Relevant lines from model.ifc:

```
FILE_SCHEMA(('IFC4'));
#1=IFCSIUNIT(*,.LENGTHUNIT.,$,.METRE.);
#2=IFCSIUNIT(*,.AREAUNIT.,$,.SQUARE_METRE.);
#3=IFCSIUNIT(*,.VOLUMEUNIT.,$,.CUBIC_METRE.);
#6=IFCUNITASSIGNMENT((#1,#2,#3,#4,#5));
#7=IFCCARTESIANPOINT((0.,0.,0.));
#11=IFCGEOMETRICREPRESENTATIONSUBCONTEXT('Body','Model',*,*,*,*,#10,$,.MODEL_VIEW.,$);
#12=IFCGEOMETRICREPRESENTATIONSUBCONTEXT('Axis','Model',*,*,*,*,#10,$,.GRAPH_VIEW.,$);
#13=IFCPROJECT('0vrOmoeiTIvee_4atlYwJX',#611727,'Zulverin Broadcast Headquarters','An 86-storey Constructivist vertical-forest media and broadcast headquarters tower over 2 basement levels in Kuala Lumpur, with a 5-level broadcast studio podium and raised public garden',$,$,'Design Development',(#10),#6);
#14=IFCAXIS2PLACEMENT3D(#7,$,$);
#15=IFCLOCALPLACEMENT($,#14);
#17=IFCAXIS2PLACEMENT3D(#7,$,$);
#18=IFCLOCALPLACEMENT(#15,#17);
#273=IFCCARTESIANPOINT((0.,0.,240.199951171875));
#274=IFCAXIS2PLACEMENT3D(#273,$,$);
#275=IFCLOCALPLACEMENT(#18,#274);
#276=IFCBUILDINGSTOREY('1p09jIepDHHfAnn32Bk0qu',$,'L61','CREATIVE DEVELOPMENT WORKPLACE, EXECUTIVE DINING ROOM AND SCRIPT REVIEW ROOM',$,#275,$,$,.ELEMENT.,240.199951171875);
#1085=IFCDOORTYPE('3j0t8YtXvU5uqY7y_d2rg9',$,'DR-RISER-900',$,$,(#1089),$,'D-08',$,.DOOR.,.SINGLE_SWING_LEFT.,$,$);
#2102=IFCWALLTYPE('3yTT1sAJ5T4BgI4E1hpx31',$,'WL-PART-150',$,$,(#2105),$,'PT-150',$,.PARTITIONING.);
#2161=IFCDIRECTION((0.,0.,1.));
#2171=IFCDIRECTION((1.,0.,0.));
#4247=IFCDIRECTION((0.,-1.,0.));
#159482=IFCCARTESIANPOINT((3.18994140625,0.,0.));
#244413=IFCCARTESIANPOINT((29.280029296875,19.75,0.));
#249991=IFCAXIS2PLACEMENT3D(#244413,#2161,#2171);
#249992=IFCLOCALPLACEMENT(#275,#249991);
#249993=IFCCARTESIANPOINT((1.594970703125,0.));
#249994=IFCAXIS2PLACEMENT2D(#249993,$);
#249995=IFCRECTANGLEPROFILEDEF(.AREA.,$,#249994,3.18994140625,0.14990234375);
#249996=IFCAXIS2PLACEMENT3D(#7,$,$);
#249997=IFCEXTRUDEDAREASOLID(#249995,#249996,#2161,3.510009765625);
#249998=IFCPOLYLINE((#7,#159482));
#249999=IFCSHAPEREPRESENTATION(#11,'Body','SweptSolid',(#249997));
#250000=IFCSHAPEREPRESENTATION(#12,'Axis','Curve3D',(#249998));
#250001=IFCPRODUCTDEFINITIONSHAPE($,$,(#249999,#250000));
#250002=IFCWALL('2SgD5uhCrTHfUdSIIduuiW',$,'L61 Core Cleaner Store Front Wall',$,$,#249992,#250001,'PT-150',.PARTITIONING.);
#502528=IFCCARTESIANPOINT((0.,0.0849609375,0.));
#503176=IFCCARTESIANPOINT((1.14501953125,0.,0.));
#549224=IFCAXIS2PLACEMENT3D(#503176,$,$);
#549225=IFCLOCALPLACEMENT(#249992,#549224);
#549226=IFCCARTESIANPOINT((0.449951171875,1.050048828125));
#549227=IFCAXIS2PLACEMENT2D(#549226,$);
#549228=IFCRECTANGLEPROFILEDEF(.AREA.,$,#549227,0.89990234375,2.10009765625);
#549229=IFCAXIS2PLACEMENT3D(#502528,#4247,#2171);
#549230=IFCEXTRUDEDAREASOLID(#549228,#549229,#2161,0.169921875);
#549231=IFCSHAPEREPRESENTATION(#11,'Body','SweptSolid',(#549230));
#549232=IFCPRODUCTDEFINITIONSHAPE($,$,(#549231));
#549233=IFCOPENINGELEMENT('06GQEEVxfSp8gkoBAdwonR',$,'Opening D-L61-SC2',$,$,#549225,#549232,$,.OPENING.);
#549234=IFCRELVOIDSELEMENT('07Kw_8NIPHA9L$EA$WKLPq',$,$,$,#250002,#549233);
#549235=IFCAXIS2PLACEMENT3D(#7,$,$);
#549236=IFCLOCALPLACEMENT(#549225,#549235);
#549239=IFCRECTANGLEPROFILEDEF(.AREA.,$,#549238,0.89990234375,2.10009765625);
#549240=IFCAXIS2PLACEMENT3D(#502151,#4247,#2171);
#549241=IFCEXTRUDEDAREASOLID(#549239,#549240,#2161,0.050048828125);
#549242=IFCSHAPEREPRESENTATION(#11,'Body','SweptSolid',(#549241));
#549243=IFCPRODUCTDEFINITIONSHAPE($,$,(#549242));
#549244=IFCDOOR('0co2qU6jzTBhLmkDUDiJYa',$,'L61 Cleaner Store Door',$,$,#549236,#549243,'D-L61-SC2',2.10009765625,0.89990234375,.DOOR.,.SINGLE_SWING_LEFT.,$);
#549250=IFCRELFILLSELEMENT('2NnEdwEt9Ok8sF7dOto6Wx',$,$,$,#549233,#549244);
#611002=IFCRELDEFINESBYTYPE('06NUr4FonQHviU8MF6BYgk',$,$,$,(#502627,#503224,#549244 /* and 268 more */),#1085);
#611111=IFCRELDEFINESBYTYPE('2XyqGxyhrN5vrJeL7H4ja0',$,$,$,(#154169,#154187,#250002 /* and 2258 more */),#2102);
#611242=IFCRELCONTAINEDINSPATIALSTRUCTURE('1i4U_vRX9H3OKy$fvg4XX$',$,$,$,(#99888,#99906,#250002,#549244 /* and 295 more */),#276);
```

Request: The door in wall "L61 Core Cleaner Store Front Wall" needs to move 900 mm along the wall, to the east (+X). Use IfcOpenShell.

```python
import ifcopenshell
import ifcopenshell.api.geometry
import ifcopenshell.util.placement
import ifcopenshell.util.unit

model = ifcopenshell.open("model.ifc")
unit_scale = ifcopenshell.util.unit.calculate_unit_scale(model)

door = model.by_guid("0co2qU6jzTBhLmkDUDiJYa")
opening = door.FillsVoids[0].RelatingOpeningElement
wall = opening.VoidsElements[0].RelatingBuildingElement

wall_matrix = ifcopenshell.util.placement.get_local_placement(wall.ObjectPlacement)
shift = wall_matrix[:3, 0] * 0.9 / unit_scale
before = ifcopenshell.util.placement.get_local_placement(door.ObjectPlacement)[:3, 3].copy()

# The door is placed relative to its opening, so it follows when the opening moves.
matrix = ifcopenshell.util.placement.get_local_placement(opening.ObjectPlacement)
matrix[:3, 3] += shift
ifcopenshell.api.geometry.edit_object_placement(
    model, product=opening, matrix=matrix, is_si=False, should_transform_children=True
)

after = ifcopenshell.util.placement.get_local_placement(door.ObjectPlacement)[:3, 3]
print("door moved by", (after - before).round(3) + 0.0)

model.write("model_edited.ifc")
```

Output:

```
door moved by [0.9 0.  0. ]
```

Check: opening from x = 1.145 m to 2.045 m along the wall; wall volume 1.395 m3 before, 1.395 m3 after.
